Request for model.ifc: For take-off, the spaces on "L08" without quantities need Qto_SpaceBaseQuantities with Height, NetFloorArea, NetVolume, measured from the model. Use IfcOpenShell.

First a look at what the model holds.

```python
import ifcopenshell
import ifcopenshell.util.element
import ifcopenshell.util.unit

model = ifcopenshell.open("model.ifc")
print(model.schema)
for unit_type in ("LENGTHUNIT", "AREAUNIT", "VOLUMEUNIT"):
    print(unit_type, ifcopenshell.util.unit.calculate_unit_scale(model, unit_type))
storey = next(s for s in model.by_type("IfcBuildingStorey") if s.Name == "L08")
spaces = [e for e in ifcopenshell.util.element.get_decomposition(storey) if e.is_a("IfcSpace")]
for e in sorted(spaces, key=lambda e: e.id()):
    print(e.id(), e.is_a(), e.Name, list(ifcopenshell.util.element.get_psets(e, qtos_only=True)), sep=" | ")
```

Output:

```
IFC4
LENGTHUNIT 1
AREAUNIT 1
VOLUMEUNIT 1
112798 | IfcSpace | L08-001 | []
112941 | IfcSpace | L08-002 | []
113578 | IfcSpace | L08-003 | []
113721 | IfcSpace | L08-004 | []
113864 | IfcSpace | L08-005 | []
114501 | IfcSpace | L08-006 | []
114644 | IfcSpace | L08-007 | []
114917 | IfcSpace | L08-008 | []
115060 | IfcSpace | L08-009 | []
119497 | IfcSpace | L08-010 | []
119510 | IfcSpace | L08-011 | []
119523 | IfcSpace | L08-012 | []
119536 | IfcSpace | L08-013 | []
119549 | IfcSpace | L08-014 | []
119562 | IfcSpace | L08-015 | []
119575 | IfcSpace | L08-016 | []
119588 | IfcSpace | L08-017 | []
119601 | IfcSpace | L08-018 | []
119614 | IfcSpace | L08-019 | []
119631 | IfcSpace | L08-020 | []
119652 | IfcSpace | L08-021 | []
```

```python
import ifcopenshell
import ifcopenshell.api.pset
import ifcopenshell.geom
import ifcopenshell.util.element
import ifcopenshell.util.shape
import ifcopenshell.util.unit

model = ifcopenshell.open("model.ifc")
unit_scale = ifcopenshell.util.unit.calculate_unit_scale(model)
area_scale = ifcopenshell.util.unit.calculate_unit_scale(model, "AREAUNIT")
volume_scale = ifcopenshell.util.unit.calculate_unit_scale(model, "VOLUMEUNIT")
settings = ifcopenshell.geom.settings()

storey = next(s for s in model.by_type("IfcBuildingStorey") if s.Name == "L08")
spaces = [e for e in ifcopenshell.util.element.get_decomposition(storey) if e.is_a("IfcSpace")]

for e in sorted(spaces, key=lambda e: e.id()):
    if ifcopenshell.util.element.get_psets(e, qtos_only=True, should_inherit=False):
        continue
    # Geometry comes back in metres, in the element's own axes.
    shape = ifcopenshell.geom.create_shape(settings, e)
    values = {
        "Height": ifcopenshell.util.shape.get_z(shape.geometry) / unit_scale,
        "NetFloorArea": ifcopenshell.util.shape.get_footprint_area(shape.geometry) / area_scale,
        "NetVolume": ifcopenshell.util.shape.get_volume(shape.geometry) / volume_scale,
    }
    qto = ifcopenshell.api.pset.add_qto(model, product=e, name="Qto_SpaceBaseQuantities")
    ifcopenshell.api.pset.edit_qto(model, qto=qto, properties=values)
    print(e.id(), {k: round(v, 3) for k, v in values.items()})

model.write("model-out.ifc")
```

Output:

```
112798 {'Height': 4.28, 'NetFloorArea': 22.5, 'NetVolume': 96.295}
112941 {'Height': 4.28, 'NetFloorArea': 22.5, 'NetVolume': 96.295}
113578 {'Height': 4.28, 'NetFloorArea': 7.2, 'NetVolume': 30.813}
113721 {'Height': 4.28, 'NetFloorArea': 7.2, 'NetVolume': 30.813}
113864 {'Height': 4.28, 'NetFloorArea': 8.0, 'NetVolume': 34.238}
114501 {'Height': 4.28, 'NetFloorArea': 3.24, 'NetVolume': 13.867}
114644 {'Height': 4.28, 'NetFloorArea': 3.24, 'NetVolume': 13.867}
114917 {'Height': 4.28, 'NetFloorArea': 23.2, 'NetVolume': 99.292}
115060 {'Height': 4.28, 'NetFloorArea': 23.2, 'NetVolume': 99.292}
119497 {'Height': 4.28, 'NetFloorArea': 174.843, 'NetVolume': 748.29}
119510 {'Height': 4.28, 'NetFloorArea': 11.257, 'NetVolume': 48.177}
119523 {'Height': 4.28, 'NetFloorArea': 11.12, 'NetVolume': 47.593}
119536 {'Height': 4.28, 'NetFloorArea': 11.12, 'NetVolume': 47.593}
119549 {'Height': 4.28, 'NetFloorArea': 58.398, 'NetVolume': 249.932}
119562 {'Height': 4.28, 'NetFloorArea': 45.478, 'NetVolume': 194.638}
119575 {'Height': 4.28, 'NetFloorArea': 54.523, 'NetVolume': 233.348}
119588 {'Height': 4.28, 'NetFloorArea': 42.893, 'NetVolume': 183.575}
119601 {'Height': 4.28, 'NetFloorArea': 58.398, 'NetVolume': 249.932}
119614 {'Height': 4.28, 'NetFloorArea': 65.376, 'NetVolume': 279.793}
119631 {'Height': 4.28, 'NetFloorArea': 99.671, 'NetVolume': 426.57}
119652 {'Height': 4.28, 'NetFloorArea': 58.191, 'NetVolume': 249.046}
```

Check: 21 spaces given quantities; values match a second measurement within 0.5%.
